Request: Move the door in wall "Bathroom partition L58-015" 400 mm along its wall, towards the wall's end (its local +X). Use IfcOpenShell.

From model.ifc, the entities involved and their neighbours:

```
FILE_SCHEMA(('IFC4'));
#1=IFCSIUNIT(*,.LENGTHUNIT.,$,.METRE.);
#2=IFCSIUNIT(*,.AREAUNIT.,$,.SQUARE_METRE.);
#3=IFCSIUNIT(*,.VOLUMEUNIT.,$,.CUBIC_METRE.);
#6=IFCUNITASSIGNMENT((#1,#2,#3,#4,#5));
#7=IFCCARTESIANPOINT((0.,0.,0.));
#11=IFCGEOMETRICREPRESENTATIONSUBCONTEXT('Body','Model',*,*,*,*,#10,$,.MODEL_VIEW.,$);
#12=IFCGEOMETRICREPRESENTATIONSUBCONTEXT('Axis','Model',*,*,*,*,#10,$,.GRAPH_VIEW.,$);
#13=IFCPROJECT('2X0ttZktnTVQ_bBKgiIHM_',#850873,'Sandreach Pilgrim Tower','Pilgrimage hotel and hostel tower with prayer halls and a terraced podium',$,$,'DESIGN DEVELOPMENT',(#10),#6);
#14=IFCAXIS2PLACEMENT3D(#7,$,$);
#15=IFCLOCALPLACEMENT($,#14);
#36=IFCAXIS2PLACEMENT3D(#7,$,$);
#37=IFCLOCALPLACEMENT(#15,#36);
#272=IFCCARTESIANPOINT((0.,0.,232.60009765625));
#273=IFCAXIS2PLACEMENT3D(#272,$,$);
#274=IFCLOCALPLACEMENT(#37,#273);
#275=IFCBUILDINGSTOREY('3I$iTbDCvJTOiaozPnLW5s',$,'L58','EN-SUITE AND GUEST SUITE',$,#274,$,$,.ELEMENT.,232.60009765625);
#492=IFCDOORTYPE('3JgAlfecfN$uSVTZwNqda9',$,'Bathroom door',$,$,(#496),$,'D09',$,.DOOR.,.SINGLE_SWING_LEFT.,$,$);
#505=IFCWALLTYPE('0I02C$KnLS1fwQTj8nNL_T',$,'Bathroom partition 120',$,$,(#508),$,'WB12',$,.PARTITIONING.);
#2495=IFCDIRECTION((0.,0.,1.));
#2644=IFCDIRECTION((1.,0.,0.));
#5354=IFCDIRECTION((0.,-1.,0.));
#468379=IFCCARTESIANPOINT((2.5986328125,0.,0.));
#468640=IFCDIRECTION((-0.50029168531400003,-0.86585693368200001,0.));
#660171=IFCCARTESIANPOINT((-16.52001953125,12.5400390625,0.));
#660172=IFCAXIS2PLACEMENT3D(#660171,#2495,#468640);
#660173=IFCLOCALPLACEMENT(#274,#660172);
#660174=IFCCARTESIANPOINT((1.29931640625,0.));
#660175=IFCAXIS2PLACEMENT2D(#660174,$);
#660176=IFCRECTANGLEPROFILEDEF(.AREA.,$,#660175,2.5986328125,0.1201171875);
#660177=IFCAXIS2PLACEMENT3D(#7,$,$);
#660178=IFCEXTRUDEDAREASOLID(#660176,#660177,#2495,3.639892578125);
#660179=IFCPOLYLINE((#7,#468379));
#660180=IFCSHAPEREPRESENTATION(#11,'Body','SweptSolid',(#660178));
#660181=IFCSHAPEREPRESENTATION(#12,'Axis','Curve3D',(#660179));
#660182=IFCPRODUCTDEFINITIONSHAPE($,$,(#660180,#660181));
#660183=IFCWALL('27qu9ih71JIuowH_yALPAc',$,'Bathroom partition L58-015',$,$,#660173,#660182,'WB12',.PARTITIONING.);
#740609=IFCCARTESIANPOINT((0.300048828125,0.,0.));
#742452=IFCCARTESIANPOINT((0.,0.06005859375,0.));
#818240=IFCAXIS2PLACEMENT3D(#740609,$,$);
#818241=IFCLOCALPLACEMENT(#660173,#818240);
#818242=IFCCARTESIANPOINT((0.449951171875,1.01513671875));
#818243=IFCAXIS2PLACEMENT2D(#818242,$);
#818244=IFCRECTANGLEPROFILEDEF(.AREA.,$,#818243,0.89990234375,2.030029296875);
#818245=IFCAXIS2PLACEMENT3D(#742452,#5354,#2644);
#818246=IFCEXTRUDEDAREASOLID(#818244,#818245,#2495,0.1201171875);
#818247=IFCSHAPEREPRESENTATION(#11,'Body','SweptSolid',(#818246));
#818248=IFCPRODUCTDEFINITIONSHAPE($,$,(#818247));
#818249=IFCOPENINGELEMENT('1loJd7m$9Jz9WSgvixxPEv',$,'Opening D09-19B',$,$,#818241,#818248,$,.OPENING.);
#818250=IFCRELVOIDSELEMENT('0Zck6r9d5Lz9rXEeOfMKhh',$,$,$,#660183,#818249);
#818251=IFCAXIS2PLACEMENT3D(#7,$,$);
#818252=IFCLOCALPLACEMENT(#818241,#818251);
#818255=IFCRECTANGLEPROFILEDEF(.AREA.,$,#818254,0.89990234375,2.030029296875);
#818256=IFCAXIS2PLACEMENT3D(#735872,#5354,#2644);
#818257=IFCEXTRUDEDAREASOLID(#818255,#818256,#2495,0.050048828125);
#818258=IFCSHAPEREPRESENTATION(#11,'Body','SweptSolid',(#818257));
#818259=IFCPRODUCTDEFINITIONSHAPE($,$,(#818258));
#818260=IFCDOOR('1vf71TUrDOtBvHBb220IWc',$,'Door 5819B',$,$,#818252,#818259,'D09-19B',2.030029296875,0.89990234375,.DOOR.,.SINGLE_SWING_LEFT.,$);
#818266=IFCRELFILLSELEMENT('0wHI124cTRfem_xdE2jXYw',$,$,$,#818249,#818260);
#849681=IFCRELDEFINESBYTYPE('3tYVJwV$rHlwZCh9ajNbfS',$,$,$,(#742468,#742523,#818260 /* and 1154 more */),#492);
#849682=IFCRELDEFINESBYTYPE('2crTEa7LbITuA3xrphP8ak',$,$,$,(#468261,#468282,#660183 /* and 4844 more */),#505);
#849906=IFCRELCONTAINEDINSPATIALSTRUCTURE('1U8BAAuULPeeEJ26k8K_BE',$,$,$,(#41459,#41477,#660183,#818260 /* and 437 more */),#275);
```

```python
import ifcopenshell
import ifcopenshell.api.geometry
import ifcopenshell.util.placement

model = ifcopenshell.open("model.ifc")

door = model.by_guid("1vf71TUrDOtBvHBb220IWc")
opening = door.FillsVoids[0].RelatingOpeningElement
wall = opening.VoidsElements[0].RelatingBuildingElement

wall_matrix = ifcopenshell.util.placement.get_local_placement(wall.ObjectPlacement)
shift = wall_matrix[:3, 0] * 0.4
before = ifcopenshell.util.placement.get_local_placement(door.ObjectPlacement)[:3, 3].copy()

# The door is placed relative to its opening, so it follows when the opening moves.
matrix = ifcopenshell.util.placement.get_local_placement(opening.ObjectPlacement)
matrix[:3, 3] += shift
ifcopenshell.api.geometry.edit_object_placement(
    model, product=opening, matrix=matrix, is_si=False, should_transform_children=True
)

after = ifcopenshell.util.placement.get_local_placement(door.ObjectPlacement)[:3, 3]
print("door moved by", (after - before).round(3) + 0.0)

model.write("model-out.ifc")
```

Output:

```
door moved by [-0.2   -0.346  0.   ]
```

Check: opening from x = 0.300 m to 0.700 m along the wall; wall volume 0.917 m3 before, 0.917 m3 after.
